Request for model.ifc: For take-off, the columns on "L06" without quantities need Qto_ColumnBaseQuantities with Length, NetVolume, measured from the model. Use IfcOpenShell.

First a look at what the model holds.

```python
import ifcopenshell
import ifcopenshell.util.element
import ifcopenshell.util.unit

model = ifcopenshell.open("model.ifc")
print(model.schema)
for unit_type in ("LENGTHUNIT", "AREAUNIT", "VOLUMEUNIT"):
    print(unit_type, ifcopenshell.util.unit.calculate_unit_scale(model, unit_type))
storey = next(s for s in model.by_type("IfcBuildingStorey") if s.Name == "L06")
columns = [e for e in ifcopenshell.util.element.get_decomposition(storey) if e.is_a("IfcColumn")]
for e in sorted(columns, key=lambda e: e.id()):
    print(e.id(), e.is_a(), e.Name, list(ifcopenshell.util.element.get_psets(e, qtos_only=True)), sep=" | ")
```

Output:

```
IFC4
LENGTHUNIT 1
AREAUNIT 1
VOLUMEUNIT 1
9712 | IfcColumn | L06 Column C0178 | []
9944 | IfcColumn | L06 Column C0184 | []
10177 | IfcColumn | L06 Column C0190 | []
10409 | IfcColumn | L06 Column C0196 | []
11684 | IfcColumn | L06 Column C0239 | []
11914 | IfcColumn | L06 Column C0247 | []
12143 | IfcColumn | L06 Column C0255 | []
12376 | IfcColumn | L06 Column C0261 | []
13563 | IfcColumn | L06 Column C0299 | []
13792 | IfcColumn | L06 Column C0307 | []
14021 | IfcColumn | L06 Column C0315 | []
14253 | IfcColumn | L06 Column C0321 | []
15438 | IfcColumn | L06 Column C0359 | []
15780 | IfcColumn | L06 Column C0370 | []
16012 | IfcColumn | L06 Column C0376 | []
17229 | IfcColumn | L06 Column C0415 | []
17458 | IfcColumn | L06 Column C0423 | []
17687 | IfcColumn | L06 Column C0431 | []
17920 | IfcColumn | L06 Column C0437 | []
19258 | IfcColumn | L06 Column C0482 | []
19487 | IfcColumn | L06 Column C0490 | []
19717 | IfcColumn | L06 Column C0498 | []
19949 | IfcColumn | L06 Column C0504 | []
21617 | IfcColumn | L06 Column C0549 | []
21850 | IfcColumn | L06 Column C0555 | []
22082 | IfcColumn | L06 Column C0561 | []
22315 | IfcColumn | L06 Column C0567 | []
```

```python
import ifcopenshell
import ifcopenshell.api.pset
import ifcopenshell.geom
import ifcopenshell.util.element
import ifcopenshell.util.shape
import ifcopenshell.util.unit

model = ifcopenshell.open("model.ifc")
unit_scale = ifcopenshell.util.unit.calculate_unit_scale(model)
volume_scale = ifcopenshell.util.unit.calculate_unit_scale(model, "VOLUMEUNIT")
settings = ifcopenshell.geom.settings()

storey = next(s for s in model.by_type("IfcBuildingStorey") if s.Name == "L06")
columns = [e for e in ifcopenshell.util.element.get_decomposition(storey) if e.is_a("IfcColumn")]

for e in sorted(columns, key=lambda e: e.id()):
    if ifcopenshell.util.element.get_psets(e, qtos_only=True, should_inherit=False):
        continue
    # Geometry comes back in metres, in the element's own axes.
    shape = ifcopenshell.geom.create_shape(settings, e)
    values = {
        "Length": ifcopenshell.util.shape.get_z(shape.geometry) / unit_scale,
        "NetVolume": ifcopenshell.util.shape.get_volume(shape.geometry) / volume_scale,
    }
    qto = ifcopenshell.api.pset.add_qto(model, product=e, name="Qto_ColumnBaseQuantities")
    ifcopenshell.api.pset.edit_qto(model, qto=qto, properties=values)
    print(e.id(), {k: round(v, 3) for k, v in values.items()})

model.write("model_rev.ifc")
```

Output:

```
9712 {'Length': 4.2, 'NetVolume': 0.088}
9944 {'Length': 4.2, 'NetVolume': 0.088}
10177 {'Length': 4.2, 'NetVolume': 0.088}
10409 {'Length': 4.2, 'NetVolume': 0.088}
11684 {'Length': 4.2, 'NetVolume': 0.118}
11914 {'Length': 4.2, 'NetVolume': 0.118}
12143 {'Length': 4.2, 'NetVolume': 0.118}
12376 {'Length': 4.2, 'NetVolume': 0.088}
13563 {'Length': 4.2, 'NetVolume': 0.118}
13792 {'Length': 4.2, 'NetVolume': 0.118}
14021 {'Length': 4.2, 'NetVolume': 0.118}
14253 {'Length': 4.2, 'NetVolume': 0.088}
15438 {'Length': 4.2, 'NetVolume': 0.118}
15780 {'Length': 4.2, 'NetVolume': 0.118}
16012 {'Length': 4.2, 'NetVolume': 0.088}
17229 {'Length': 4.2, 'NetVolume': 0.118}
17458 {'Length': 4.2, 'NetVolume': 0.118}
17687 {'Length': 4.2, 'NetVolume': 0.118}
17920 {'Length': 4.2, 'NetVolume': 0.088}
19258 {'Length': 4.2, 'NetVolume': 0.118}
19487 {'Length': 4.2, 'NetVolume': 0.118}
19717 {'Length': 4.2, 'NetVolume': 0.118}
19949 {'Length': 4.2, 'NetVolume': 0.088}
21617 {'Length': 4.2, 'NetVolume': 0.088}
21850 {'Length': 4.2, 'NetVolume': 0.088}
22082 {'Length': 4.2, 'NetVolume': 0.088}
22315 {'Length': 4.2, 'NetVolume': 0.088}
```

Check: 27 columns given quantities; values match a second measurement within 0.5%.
